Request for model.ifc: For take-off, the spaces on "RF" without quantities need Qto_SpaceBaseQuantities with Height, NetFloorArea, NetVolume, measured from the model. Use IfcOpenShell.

First a look at what the model holds.

```python
import ifcopenshell
import ifcopenshell.util.element
import ifcopenshell.util.unit

model = ifcopenshell.open("model.ifc")
print(model.schema)
for unit_type in ("LENGTHUNIT", "AREAUNIT", "VOLUMEUNIT"):
    print(unit_type, ifcopenshell.util.unit.calculate_unit_scale(model, unit_type))
storey = next(s for s in model.by_type("IfcBuildingStorey") if s.Name == "RF")
spaces = [e for e in ifcopenshell.util.element.get_decomposition(storey) if e.is_a("IfcSpace")]
for e in sorted(spaces, key=lambda e: e.id()):
    print(e.id(), e.is_a(), e.Name, list(ifcopenshell.util.element.get_psets(e, qtos_only=True)), sep=" | ")
```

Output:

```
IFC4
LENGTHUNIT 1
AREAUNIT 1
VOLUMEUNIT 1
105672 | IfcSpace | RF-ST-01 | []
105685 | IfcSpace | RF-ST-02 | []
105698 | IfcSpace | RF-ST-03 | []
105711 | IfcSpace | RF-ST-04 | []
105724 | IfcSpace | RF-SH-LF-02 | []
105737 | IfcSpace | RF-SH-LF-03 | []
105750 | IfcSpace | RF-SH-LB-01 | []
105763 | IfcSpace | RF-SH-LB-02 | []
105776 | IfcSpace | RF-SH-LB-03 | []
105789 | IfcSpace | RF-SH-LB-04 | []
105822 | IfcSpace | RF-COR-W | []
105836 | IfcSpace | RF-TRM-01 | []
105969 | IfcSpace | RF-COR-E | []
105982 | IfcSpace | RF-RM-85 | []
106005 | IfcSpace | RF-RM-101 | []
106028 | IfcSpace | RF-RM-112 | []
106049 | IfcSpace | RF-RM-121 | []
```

```python
import ifcopenshell
import ifcopenshell.api.pset
import ifcopenshell.geom
import ifcopenshell.util.element
import ifcopenshell.util.shape
import ifcopenshell.util.unit

model = ifcopenshell.open("model.ifc")
unit_scale = ifcopenshell.util.unit.calculate_unit_scale(model)
area_scale = ifcopenshell.util.unit.calculate_unit_scale(model, "AREAUNIT")
volume_scale = ifcopenshell.util.unit.calculate_unit_scale(model, "VOLUMEUNIT")
settings = ifcopenshell.geom.settings()

storey = next(s for s in model.by_type("IfcBuildingStorey") if s.Name == "RF")
spaces = [e for e in ifcopenshell.util.element.get_decomposition(storey) if e.is_a("IfcSpace")]

for e in sorted(spaces, key=lambda e: e.id()):
    if ifcopenshell.util.element.get_psets(e, qtos_only=True, should_inherit=False):
        continue
    # Geometry comes back in metres, in the element's own axes.
    shape = ifcopenshell.geom.create_shape(settings, e)
    values = {
        "Height": ifcopenshell.util.shape.get_z(shape.geometry) / unit_scale,
        "NetFloorArea": ifcopenshell.util.shape.get_footprint_area(shape.geometry) / area_scale,
        "NetVolume": ifcopenshell.util.shape.get_volume(shape.geometry) / volume_scale,
    }
    qto = ifcopenshell.api.pset.add_qto(model, product=e, name="Qto_SpaceBaseQuantities")
    ifcopenshell.api.pset.edit_qto(model, qto=qto, properties=values)
    print(e.id(), {k: round(v, 3) for k, v in values.items()})

model.write("model-out.ifc")
```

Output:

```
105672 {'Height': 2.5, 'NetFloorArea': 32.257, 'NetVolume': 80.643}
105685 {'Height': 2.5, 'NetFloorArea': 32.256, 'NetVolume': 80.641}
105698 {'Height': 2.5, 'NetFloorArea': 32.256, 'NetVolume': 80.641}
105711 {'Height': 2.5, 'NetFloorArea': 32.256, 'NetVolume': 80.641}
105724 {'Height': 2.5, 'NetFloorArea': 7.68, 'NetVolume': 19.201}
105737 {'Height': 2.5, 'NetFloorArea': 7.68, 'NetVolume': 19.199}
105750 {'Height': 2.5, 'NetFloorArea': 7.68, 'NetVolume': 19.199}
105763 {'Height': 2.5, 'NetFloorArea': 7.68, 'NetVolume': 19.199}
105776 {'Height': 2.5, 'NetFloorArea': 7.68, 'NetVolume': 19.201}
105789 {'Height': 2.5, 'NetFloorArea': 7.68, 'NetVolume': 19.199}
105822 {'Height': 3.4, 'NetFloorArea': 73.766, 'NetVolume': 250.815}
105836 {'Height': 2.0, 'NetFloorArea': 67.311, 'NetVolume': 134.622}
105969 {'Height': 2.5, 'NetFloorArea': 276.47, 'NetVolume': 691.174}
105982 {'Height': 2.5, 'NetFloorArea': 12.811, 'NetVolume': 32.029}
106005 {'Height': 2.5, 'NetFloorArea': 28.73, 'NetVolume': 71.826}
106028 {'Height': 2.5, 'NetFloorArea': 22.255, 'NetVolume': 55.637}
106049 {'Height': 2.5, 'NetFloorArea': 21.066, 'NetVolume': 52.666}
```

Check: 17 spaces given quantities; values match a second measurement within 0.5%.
